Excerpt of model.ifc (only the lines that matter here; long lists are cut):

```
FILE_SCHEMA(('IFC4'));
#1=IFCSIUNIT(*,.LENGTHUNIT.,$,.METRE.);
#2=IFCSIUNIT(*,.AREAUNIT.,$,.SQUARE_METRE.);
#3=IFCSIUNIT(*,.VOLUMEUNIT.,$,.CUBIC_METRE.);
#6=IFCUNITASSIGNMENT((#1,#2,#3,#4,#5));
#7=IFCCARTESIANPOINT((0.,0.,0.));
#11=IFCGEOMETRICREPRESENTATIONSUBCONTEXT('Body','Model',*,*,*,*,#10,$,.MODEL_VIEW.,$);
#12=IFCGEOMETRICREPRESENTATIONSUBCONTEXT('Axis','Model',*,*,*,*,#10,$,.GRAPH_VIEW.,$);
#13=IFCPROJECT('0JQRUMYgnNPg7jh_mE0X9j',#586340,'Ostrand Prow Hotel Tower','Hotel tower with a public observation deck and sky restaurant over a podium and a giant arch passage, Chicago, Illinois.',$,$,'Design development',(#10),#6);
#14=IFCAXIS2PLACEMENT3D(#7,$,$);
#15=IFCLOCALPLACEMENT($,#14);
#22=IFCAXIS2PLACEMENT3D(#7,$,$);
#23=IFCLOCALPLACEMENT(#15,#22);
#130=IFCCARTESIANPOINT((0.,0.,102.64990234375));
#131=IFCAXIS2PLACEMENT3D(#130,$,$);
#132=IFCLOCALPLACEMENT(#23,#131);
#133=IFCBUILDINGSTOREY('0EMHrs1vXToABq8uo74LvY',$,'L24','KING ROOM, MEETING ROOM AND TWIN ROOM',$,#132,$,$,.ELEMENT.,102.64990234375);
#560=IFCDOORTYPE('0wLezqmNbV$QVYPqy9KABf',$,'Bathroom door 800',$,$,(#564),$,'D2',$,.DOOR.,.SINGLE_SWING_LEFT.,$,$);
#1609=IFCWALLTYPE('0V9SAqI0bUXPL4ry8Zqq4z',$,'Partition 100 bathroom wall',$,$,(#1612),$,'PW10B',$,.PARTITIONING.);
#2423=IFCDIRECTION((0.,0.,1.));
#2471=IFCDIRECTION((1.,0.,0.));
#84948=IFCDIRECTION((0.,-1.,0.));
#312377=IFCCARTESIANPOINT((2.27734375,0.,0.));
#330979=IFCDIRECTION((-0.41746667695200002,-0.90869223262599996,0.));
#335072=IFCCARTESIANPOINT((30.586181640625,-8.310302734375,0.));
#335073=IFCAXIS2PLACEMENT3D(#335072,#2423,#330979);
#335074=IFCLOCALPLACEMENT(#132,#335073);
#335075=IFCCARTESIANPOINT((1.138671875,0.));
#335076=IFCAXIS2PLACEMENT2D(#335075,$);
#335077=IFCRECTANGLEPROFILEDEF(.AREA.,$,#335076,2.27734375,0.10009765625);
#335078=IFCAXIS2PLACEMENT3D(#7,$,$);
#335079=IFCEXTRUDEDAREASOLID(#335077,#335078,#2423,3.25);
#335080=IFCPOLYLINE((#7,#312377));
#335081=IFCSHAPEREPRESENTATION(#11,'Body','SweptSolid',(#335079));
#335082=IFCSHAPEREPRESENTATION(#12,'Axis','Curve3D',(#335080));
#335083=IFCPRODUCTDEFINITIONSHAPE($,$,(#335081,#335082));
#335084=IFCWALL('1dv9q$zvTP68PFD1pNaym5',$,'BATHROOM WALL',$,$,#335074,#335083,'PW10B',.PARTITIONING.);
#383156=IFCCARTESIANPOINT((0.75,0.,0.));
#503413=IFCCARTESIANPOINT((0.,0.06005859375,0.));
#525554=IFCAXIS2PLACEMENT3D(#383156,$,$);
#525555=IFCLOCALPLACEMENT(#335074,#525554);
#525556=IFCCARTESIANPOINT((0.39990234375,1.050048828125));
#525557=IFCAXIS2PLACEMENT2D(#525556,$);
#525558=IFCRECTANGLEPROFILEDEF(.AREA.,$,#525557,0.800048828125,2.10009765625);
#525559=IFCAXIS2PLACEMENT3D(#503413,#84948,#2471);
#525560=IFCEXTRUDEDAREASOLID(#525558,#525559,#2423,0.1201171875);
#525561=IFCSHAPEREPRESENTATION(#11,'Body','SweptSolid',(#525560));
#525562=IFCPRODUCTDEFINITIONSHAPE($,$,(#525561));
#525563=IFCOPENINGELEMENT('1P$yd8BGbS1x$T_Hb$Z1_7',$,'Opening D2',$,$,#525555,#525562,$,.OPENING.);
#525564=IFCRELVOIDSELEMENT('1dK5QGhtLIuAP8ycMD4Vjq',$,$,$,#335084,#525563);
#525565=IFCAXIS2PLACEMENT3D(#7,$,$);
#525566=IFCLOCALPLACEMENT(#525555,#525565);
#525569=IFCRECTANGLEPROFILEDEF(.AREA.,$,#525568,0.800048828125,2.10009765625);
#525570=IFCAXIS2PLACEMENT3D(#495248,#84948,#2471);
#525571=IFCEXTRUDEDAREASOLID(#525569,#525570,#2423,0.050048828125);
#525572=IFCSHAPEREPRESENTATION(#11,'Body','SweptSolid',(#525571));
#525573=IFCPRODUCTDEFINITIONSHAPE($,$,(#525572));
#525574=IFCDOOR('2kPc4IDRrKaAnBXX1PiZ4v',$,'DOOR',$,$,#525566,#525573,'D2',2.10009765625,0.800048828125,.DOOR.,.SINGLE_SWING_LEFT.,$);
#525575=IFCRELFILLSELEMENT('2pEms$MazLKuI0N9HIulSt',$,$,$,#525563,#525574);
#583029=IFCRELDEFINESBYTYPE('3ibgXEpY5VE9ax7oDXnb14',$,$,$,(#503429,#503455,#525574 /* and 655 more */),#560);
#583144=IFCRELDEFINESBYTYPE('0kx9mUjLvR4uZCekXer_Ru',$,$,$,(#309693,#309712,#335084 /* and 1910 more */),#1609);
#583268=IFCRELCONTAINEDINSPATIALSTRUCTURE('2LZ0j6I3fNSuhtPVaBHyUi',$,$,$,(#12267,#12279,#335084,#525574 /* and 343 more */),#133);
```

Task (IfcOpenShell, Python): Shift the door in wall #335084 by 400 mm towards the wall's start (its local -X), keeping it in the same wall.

```python
import ifcopenshell
import ifcopenshell.api.geometry
import ifcopenshell.util.placement

model = ifcopenshell.open("model.ifc")

door = model.by_guid("2kPc4IDRrKaAnBXX1PiZ4v")
opening = door.FillsVoids[0].RelatingOpeningElement
wall = opening.VoidsElements[0].RelatingBuildingElement

wall_matrix = ifcopenshell.util.placement.get_local_placement(wall.ObjectPlacement)
shift = wall_matrix[:3, 0] * -0.4
before = ifcopenshell.util.placement.get_local_placement(door.ObjectPlacement)[:3, 3].copy()

# The door is placed relative to its opening, so it follows when the opening moves.
matrix = ifcopenshell.util.placement.get_local_placement(opening.ObjectPlacement)
matrix[:3, 3] += shift
ifcopenshell.api.geometry.edit_object_placement(
    model, product=opening, matrix=matrix, is_si=False, should_transform_children=True
)

after = ifcopenshell.util.placement.get_local_placement(door.ObjectPlacement)[:3, 3]
print("door moved by", (after - before).round(3) + 0.0)

model.write("model_edited.ifc")
```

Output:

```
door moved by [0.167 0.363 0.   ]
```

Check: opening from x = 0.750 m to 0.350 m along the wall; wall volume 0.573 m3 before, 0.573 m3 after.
